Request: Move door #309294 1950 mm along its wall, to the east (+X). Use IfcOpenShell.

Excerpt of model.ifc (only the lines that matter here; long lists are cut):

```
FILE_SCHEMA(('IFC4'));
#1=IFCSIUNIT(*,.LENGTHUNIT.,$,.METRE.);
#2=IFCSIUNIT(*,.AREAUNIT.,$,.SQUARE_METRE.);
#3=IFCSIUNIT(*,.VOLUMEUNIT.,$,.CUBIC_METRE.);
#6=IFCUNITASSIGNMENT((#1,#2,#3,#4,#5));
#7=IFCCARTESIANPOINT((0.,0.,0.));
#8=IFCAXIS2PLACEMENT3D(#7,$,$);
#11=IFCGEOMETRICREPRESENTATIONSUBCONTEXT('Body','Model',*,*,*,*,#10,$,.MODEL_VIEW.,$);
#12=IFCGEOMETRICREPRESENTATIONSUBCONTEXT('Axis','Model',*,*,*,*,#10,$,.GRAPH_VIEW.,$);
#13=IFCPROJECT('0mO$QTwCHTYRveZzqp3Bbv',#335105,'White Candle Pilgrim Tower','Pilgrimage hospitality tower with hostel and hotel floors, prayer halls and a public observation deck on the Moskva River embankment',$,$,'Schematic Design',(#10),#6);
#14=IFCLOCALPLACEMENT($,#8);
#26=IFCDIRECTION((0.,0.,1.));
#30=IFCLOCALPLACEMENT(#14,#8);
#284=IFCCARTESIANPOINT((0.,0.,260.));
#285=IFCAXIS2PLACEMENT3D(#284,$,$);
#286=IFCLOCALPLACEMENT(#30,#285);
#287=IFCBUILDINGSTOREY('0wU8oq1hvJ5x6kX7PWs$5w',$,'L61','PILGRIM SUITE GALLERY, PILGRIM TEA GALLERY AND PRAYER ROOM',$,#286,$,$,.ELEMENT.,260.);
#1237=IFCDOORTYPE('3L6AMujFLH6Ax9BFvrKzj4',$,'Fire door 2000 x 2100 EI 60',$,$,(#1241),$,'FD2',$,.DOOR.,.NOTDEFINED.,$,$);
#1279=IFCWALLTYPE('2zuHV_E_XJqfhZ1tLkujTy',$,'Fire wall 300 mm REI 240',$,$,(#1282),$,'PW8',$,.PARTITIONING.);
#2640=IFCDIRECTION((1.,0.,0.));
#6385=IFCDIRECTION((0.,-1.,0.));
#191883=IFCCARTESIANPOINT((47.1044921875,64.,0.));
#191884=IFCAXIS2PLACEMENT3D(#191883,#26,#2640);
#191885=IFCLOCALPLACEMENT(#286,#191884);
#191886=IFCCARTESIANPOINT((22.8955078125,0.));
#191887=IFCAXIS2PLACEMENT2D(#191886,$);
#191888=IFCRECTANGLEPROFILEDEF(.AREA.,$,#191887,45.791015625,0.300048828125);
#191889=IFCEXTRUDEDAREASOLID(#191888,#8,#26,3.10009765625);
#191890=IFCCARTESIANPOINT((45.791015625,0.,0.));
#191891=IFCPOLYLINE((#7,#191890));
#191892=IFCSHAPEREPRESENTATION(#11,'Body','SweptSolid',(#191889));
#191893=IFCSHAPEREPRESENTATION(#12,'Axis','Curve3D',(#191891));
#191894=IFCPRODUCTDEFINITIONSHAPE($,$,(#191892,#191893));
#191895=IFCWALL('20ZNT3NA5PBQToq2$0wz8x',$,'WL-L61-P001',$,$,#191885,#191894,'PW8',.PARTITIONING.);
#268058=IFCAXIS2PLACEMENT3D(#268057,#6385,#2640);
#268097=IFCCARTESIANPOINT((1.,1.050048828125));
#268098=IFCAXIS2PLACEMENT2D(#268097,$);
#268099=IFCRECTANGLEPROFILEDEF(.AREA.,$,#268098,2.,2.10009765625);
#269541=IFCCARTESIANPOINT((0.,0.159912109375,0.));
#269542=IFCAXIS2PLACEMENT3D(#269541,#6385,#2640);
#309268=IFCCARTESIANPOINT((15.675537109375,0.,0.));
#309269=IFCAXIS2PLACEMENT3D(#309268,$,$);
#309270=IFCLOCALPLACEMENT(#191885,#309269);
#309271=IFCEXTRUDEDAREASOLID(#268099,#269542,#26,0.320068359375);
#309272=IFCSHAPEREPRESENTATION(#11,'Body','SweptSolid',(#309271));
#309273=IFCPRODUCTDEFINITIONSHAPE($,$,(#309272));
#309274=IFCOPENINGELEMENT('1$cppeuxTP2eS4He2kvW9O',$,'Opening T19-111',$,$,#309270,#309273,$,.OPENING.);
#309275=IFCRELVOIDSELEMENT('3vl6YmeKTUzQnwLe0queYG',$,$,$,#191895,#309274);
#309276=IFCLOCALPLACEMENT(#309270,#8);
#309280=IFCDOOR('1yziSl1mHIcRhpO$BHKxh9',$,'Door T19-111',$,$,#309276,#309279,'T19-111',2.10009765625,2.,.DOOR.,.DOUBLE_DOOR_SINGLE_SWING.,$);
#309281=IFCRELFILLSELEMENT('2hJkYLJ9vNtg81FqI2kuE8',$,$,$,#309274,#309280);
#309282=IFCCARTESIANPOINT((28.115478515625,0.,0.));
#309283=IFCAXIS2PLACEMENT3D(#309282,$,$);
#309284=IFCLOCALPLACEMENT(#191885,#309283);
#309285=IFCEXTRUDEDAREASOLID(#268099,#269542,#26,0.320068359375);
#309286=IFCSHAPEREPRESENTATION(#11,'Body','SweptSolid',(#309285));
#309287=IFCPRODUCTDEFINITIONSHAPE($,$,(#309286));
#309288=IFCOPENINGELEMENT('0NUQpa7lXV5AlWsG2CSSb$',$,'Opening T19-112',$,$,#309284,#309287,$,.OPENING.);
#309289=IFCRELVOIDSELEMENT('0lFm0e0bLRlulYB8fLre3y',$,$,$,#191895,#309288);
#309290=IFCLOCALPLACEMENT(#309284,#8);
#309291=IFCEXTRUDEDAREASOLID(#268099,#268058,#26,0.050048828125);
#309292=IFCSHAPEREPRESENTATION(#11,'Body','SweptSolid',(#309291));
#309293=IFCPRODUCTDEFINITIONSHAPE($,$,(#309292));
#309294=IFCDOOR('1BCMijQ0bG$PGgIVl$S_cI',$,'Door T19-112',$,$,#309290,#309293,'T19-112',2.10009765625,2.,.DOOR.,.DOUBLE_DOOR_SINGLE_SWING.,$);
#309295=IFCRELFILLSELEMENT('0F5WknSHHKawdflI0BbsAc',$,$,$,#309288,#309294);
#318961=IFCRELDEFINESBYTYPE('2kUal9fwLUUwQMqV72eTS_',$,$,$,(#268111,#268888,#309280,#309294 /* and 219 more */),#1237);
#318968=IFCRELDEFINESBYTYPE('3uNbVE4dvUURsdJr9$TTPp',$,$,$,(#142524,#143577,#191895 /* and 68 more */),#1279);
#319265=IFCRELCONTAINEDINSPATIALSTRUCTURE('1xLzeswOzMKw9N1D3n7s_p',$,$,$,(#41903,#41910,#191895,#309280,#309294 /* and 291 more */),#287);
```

```python
import ifcopenshell
import ifcopenshell.api.geometry
import ifcopenshell.util.placement
import ifcopenshell.util.unit

model = ifcopenshell.open("model.ifc")
unit_scale = ifcopenshell.util.unit.calculate_unit_scale(model)

door = model.by_guid("1BCMijQ0bG$PGgIVl$S_cI")
opening = door.FillsVoids[0].RelatingOpeningElement
wall = opening.VoidsElements[0].RelatingBuildingElement

wall_matrix = ifcopenshell.util.placement.get_local_placement(wall.ObjectPlacement)
shift = wall_matrix[:3, 0] * 1.95 / unit_scale
before = ifcopenshell.util.placement.get_local_placement(door.ObjectPlacement)[:3, 3].copy()

# The door is placed relative to its opening, so it follows when the opening moves.
matrix = ifcopenshell.util.placement.get_local_placement(opening.ObjectPlacement)
matrix[:3, 3] += shift
ifcopenshell.api.geometry.edit_object_placement(
    model, product=opening, matrix=matrix, is_si=False, should_transform_children=True
)

after = ifcopenshell.util.placement.get_local_placement(door.ObjectPlacement)[:3, 3]
print("door moved by", (after - before).round(3) + 0.0)

model.write("model_edited.ifc")
```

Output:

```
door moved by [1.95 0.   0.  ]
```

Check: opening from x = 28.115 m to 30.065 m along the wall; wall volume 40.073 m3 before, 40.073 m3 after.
